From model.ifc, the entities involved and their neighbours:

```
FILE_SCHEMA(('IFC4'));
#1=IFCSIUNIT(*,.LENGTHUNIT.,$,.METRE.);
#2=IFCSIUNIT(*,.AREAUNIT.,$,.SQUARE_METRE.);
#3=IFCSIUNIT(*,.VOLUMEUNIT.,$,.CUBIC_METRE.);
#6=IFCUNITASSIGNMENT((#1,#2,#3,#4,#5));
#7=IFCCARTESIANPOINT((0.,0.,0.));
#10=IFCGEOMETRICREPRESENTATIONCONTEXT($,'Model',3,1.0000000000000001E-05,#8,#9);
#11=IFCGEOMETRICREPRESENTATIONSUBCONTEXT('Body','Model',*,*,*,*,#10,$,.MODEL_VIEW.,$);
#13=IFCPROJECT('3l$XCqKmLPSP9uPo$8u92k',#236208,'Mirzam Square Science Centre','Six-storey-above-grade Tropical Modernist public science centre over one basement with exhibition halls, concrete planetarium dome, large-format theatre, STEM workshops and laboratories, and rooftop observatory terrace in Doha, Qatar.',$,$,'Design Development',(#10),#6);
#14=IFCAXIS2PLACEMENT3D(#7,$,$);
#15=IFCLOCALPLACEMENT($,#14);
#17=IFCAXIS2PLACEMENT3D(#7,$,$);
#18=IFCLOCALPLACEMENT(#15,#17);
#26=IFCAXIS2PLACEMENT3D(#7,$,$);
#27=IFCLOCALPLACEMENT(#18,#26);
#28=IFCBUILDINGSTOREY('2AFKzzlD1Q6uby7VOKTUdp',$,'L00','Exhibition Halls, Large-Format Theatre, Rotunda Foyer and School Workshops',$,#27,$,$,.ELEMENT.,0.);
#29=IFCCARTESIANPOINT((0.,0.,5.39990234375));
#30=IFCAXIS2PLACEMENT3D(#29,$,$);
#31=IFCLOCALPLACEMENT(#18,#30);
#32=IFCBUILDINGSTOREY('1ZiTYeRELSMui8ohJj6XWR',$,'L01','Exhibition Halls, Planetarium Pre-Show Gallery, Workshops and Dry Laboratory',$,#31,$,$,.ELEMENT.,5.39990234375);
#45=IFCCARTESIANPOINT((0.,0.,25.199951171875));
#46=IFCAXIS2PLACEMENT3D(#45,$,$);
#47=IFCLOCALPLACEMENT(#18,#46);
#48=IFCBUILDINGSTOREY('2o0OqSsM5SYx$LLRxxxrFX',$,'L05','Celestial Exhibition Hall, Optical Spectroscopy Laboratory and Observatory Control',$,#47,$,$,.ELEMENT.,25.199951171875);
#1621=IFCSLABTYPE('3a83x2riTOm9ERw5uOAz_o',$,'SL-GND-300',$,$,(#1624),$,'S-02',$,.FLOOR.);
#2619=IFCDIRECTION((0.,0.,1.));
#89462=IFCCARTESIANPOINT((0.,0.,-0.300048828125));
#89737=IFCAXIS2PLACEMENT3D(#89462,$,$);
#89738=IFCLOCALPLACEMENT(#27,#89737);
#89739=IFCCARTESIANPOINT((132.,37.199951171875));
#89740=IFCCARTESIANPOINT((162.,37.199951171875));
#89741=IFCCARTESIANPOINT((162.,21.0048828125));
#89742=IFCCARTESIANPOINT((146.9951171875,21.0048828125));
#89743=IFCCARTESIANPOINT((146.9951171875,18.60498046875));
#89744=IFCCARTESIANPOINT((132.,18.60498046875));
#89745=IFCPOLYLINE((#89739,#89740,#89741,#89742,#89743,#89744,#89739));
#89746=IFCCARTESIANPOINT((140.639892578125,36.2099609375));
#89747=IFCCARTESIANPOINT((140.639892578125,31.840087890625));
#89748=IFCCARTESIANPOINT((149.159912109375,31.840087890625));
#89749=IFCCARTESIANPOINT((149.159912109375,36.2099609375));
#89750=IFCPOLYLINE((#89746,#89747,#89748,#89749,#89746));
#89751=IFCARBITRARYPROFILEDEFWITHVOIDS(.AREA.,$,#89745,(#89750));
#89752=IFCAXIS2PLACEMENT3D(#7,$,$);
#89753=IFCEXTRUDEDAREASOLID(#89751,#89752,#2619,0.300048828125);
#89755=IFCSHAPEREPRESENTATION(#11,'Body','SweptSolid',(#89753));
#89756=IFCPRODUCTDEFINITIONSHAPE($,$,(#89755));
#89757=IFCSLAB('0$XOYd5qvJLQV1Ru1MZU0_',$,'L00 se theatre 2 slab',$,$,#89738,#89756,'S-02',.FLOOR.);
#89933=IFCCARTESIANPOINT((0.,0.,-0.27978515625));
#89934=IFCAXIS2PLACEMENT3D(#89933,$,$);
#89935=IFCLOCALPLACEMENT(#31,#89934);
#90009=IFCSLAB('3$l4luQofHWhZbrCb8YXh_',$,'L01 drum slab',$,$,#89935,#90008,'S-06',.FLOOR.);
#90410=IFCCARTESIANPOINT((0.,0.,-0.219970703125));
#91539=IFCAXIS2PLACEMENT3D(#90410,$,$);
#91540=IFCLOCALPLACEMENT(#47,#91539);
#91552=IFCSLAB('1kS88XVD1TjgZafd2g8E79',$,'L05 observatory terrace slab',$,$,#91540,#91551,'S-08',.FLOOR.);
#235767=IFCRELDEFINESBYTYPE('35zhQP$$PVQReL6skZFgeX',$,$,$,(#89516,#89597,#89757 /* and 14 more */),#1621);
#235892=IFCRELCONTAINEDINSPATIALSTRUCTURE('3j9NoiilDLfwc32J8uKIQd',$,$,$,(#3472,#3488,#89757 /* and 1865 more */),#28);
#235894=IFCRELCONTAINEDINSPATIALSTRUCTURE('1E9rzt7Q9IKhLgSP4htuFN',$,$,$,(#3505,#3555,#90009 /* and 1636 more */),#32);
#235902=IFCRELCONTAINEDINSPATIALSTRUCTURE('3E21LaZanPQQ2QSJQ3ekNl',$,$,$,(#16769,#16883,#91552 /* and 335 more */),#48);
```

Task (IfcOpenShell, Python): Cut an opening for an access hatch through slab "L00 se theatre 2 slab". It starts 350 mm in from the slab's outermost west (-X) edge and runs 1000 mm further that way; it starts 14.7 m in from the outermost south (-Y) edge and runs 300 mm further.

```python
import numpy as np
import ifcopenshell
import ifcopenshell.api.feature
import ifcopenshell.api.geometry
import ifcopenshell.api.root
import ifcopenshell.geom
import ifcopenshell.util.placement
import ifcopenshell.util.representation
import ifcopenshell.util.shape
import ifcopenshell.util.unit

model = ifcopenshell.open("model.ifc")
unit_scale = ifcopenshell.util.unit.calculate_unit_scale(model)
settings = ifcopenshell.geom.settings()


def volume(element):
    """Net volume in cubic metres, openings subtracted."""
    shape = ifcopenshell.geom.create_shape(settings, element)
    return ifcopenshell.util.shape.get_volume(shape.geometry)


slab = model.by_guid("0$XOYd5qvJLQV1Ru1MZU0_")
before = volume(slab)

# Extent in the slab's own axes, in metres. The edges named are its -X and -Y sides.
slab_shape = ifcopenshell.geom.create_shape(settings, slab)
vertices = ifcopenshell.util.shape.get_vertices(slab_shape.geometry)
x_min, y_min, bottom = vertices.min(axis=0)
top = vertices[:, 2].max()

opening = ifcopenshell.api.root.create_entity(model, ifc_class="IfcOpeningElement", name="Access hatch opening", predefined_type="OPENING")
context = ifcopenshell.util.representation.get_context(model, "Model", "Body", "MODEL_VIEW")
width, depth = 1, 0.3
outline = [(0.0, 0.0), (width, 0.0), (width, depth), (0.0, depth), (0.0, 0.0)]
# Overshoot both faces by 50 mm so the cut is clean.
shape = ifcopenshell.api.geometry.add_slab_representation(
    model, context=context, depth=top - bottom + 0.1, polyline=outline
)
ifcopenshell.api.geometry.assign_representation(model, product=opening, representation=shape)

matrix = ifcopenshell.util.placement.get_local_placement(slab.ObjectPlacement)
matrix[:, 3] = matrix @ np.append(np.array([x_min + 0.35, y_min + 14.7, bottom - 0.05]) / unit_scale, 1.0)
ifcopenshell.api.geometry.edit_object_placement(model, product=opening, matrix=matrix, is_si=False)
ifcopenshell.api.feature.add_feature(model, feature=opening, element=slab)

after = volume(slab)

print(f"slab volume {before:.3f} -> {after:.3f} m3")

model.write("model_edited.ifc")
```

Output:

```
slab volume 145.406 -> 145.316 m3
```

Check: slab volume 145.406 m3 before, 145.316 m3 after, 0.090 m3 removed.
